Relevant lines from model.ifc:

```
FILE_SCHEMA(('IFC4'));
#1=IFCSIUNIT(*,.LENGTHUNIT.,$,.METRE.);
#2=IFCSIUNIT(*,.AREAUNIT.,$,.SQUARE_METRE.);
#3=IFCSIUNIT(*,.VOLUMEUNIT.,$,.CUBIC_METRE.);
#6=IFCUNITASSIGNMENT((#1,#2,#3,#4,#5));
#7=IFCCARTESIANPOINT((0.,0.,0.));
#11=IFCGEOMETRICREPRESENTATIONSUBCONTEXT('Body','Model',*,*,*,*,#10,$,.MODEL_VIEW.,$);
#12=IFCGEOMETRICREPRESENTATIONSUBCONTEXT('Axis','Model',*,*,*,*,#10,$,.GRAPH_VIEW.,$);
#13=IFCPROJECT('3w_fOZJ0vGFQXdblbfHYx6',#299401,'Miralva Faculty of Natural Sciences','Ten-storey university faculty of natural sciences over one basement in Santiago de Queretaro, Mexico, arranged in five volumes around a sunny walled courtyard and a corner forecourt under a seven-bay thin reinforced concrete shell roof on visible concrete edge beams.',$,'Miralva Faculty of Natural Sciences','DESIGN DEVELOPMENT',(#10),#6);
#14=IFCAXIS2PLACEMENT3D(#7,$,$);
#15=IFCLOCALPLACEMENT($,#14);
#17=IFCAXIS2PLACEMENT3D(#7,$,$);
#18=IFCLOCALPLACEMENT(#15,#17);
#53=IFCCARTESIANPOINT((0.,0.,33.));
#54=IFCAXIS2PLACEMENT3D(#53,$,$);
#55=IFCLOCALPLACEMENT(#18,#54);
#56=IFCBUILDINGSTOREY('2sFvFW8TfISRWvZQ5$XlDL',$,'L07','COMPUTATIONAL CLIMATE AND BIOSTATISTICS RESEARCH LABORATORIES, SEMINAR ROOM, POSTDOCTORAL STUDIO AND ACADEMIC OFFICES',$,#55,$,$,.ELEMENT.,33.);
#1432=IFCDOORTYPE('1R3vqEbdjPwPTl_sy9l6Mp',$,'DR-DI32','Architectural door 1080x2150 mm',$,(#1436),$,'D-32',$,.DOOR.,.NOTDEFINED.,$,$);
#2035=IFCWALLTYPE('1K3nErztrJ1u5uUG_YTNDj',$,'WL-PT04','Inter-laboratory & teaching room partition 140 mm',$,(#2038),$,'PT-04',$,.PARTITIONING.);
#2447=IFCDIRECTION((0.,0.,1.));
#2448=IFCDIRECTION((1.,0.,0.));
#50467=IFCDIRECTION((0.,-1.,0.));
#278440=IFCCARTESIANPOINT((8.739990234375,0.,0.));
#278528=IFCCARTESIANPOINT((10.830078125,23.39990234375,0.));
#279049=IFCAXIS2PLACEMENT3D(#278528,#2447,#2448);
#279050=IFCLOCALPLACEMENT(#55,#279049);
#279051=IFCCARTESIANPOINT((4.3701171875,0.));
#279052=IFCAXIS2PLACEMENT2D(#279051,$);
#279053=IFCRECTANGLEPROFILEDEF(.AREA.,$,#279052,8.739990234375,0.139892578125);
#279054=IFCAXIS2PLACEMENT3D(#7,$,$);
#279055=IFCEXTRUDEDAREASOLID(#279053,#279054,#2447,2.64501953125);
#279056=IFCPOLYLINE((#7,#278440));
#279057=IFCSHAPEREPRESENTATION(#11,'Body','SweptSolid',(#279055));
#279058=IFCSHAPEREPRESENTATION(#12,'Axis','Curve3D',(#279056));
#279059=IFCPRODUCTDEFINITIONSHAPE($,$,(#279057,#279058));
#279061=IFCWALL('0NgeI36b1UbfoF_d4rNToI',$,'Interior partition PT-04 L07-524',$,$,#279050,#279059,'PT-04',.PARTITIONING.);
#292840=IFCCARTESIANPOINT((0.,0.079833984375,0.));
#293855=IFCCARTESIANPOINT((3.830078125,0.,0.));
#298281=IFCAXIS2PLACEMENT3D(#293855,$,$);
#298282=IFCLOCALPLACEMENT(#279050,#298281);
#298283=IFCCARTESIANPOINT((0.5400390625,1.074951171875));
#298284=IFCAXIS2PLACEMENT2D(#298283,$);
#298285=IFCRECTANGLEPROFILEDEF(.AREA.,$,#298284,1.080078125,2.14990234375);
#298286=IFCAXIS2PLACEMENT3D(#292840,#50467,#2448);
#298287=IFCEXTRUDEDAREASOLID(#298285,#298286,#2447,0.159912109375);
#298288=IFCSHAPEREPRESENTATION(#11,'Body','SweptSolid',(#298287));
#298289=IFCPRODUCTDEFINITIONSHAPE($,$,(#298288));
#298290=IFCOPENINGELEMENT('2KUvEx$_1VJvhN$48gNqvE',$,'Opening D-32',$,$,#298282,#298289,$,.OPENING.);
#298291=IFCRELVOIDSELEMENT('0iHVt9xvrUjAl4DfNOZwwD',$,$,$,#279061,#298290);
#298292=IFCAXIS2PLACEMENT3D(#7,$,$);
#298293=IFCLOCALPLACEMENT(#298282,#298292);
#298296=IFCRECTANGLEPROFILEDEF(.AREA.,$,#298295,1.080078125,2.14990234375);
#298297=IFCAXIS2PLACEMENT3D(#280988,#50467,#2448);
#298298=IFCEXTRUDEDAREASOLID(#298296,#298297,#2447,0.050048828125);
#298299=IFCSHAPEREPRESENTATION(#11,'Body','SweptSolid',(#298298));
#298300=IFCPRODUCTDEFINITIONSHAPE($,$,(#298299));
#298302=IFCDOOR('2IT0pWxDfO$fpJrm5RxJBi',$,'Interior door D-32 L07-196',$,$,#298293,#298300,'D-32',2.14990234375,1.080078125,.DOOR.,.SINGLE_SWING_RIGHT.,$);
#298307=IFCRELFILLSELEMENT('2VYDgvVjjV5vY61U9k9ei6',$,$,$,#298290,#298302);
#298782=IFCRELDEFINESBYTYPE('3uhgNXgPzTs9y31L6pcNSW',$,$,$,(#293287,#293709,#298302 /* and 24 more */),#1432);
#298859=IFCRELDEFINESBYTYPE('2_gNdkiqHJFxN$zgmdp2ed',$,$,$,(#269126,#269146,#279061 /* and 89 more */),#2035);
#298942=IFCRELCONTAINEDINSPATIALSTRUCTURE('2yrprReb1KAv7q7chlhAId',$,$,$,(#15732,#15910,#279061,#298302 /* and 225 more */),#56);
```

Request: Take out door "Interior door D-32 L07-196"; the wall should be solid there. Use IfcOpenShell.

```python
import ifcopenshell
import ifcopenshell.api.feature
import ifcopenshell.api.root
import ifcopenshell.geom
import ifcopenshell.util.shape

model = ifcopenshell.open("model.ifc")
settings = ifcopenshell.geom.settings()


def volume(element):
    """Net volume in cubic metres, openings subtracted."""
    shape = ifcopenshell.geom.create_shape(settings, element)
    return ifcopenshell.util.shape.get_volume(shape.geometry)


door = model.by_id(298302)
opening = door.FillsVoids[0].RelatingOpeningElement
wall = opening.VoidsElements[0].RelatingBuildingElement
before = volume(wall)

ifcopenshell.api.root.remove_product(model, product=door)
ifcopenshell.api.feature.remove_feature(model, feature=opening)

after = volume(wall)

print(f"wall volume {before:.3f} -> {after:.3f} m3")

model.write("model_edited.ifc")
```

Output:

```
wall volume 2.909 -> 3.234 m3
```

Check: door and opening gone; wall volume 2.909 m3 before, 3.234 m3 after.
